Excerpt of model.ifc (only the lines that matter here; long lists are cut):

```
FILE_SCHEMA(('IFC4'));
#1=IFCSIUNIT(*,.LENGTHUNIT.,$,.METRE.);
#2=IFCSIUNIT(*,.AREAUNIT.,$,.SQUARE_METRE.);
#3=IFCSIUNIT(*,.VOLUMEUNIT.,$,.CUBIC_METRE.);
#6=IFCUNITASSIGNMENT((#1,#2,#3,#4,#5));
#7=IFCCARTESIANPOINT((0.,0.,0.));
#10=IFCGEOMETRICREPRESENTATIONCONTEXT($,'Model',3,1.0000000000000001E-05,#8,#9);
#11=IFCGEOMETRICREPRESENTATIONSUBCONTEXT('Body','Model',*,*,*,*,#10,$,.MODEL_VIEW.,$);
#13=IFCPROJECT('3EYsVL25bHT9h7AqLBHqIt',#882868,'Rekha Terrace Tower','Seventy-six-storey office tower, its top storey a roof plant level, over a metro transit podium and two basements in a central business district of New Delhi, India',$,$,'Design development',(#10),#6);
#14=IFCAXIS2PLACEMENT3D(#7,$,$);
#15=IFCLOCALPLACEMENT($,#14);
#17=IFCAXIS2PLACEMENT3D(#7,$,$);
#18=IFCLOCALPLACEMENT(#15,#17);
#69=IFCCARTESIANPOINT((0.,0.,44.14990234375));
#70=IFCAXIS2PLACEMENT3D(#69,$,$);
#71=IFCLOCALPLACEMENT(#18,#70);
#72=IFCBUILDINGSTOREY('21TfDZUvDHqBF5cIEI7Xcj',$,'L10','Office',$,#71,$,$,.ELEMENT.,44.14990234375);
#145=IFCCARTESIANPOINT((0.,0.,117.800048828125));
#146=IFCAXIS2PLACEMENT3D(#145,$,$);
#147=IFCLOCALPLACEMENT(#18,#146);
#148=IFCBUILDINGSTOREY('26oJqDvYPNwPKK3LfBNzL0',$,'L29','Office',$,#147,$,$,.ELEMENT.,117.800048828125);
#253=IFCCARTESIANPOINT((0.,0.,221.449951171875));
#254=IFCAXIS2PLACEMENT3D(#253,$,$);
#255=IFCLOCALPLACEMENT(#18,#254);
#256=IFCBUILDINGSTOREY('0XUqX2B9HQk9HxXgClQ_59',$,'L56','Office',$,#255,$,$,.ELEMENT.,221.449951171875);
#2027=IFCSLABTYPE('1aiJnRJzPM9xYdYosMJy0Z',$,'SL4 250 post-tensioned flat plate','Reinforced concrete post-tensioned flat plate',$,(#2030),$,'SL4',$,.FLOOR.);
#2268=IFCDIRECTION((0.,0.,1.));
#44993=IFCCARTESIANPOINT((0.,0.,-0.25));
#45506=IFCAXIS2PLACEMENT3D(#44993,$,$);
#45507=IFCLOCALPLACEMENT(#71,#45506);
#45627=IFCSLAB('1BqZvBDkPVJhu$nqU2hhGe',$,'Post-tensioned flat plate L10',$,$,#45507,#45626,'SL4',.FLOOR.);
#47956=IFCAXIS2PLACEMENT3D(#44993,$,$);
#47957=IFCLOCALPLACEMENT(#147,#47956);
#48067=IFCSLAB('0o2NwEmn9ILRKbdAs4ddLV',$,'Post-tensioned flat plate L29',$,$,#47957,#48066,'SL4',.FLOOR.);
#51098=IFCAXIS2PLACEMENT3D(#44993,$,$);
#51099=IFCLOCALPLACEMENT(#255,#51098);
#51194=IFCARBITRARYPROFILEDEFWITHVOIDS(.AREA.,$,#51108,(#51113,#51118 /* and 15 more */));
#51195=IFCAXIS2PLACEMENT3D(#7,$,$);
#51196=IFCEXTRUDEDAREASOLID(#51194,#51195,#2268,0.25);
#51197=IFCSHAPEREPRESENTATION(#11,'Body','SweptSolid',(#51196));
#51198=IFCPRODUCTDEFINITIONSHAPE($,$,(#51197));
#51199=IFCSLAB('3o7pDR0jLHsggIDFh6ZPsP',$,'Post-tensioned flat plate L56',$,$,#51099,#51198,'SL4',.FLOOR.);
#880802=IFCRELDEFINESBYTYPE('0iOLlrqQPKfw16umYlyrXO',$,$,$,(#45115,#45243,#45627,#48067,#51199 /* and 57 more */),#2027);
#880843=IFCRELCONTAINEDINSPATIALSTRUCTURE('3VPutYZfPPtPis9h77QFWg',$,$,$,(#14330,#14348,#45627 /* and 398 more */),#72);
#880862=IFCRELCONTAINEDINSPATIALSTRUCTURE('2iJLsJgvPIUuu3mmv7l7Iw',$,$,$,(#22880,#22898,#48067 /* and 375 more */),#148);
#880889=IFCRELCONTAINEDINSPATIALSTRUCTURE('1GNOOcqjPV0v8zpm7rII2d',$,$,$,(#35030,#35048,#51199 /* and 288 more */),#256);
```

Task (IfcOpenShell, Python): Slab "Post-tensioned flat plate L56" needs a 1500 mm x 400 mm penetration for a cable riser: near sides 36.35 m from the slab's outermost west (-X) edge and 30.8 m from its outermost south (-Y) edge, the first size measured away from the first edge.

```python
import numpy as np
import ifcopenshell
import ifcopenshell.api.feature
import ifcopenshell.api.geometry
import ifcopenshell.api.root
import ifcopenshell.geom
import ifcopenshell.util.placement
import ifcopenshell.util.representation
import ifcopenshell.util.shape
import ifcopenshell.util.unit

model = ifcopenshell.open("model.ifc")
unit_scale = ifcopenshell.util.unit.calculate_unit_scale(model)
settings = ifcopenshell.geom.settings()


def volume(element):
    """Net volume in cubic metres, openings subtracted."""
    shape = ifcopenshell.geom.create_shape(settings, element)
    return ifcopenshell.util.shape.get_volume(shape.geometry)


slab = model.by_guid("3o7pDR0jLHsggIDFh6ZPsP")
before = volume(slab)

# Extent in the slab's own axes, in metres. The edges named are its -X and -Y sides.
slab_shape = ifcopenshell.geom.create_shape(settings, slab)
vertices = ifcopenshell.util.shape.get_vertices(slab_shape.geometry)
x_min, y_min, bottom = vertices.min(axis=0)
top = vertices[:, 2].max()

opening = ifcopenshell.api.root.create_entity(model, ifc_class="IfcOpeningElement", name="Cable riser opening", predefined_type="OPENING")
context = ifcopenshell.util.representation.get_context(model, "Model", "Body", "MODEL_VIEW")
width, depth = 1.5, 0.4
outline = [(0.0, 0.0), (width, 0.0), (width, depth), (0.0, depth), (0.0, 0.0)]
# Overshoot both faces by 50 mm so the cut is clean.
shape = ifcopenshell.api.geometry.add_slab_representation(
    model, context=context, depth=top - bottom + 0.1, polyline=outline
)
ifcopenshell.api.geometry.assign_representation(model, product=opening, representation=shape)

matrix = ifcopenshell.util.placement.get_local_placement(slab.ObjectPlacement)
matrix[:, 3] = matrix @ np.append(np.array([x_min + 36.35, y_min + 30.8, bottom - 0.05]) / unit_scale, 1.0)
ifcopenshell.api.geometry.edit_object_placement(model, product=opening, matrix=matrix, is_si=False)
ifcopenshell.api.feature.add_feature(model, feature=opening, element=slab)

after = volume(slab)

print(f"slab volume {before:.3f} -> {after:.3f} m3")

model.write("model-out.ifc")
```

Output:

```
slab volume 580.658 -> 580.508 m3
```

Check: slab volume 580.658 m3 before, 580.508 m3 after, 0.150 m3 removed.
